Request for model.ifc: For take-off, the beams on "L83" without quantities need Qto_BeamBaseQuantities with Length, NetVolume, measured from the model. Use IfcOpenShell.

First a look at what the model holds.

```python
import ifcopenshell
import ifcopenshell.util.element
import ifcopenshell.util.unit

model = ifcopenshell.open("model.ifc")
print(model.schema)
for unit_type in ("LENGTHUNIT", "AREAUNIT", "VOLUMEUNIT"):
    print(unit_type, ifcopenshell.util.unit.calculate_unit_scale(model, unit_type))
storey = next(s for s in model.by_type("IfcBuildingStorey") if s.Name == "L83")
beams = [e for e in ifcopenshell.util.element.get_decomposition(storey) if e.is_a("IfcBeam")]
for e in sorted(beams, key=lambda e: e.id()):
    print(e.id(), e.is_a(), e.Name, list(ifcopenshell.util.element.get_psets(e, qtos_only=True)), sep=" | ")
```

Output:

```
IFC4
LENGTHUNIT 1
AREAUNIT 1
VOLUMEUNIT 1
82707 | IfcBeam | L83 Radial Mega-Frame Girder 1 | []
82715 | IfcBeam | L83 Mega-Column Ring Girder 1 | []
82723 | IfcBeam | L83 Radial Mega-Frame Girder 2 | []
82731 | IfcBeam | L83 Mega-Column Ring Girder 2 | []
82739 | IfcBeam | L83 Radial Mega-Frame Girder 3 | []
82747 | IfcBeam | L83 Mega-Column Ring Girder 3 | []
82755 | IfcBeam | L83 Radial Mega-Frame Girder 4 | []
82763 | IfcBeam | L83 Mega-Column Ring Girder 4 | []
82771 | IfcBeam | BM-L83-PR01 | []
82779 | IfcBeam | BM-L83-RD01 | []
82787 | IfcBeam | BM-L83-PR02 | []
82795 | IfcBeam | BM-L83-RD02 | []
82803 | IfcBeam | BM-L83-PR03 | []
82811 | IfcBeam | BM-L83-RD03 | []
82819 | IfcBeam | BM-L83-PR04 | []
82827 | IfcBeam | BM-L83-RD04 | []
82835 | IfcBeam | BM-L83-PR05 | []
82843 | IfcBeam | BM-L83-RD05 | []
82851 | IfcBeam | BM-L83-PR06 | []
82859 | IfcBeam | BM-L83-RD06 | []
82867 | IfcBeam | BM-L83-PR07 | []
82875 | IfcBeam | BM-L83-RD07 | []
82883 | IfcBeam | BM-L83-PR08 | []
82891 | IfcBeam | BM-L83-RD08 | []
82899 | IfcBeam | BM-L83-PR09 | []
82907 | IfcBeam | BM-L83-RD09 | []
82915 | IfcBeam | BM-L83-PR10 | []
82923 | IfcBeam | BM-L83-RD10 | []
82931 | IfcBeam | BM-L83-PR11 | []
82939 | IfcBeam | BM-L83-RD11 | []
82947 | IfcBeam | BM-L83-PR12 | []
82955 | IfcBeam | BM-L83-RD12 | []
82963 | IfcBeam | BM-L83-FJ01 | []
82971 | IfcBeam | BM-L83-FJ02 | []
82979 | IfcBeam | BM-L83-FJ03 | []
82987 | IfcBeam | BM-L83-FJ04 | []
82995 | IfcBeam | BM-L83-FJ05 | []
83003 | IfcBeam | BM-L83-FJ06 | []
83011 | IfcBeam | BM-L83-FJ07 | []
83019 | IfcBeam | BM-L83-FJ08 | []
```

```python
import ifcopenshell
import ifcopenshell.api.pset
import ifcopenshell.geom
import ifcopenshell.util.element
import ifcopenshell.util.shape
import ifcopenshell.util.unit

model = ifcopenshell.open("model.ifc")
unit_scale = ifcopenshell.util.unit.calculate_unit_scale(model)
volume_scale = ifcopenshell.util.unit.calculate_unit_scale(model, "VOLUMEUNIT")
settings = ifcopenshell.geom.settings()

storey = next(s for s in model.by_type("IfcBuildingStorey") if s.Name == "L83")
beams = [e for e in ifcopenshell.util.element.get_decomposition(storey) if e.is_a("IfcBeam")]

for e in sorted(beams, key=lambda e: e.id()):
    if ifcopenshell.util.element.get_psets(e, qtos_only=True, should_inherit=False):
        continue
    # Geometry comes back in metres, in the element's own axes.
    shape = ifcopenshell.geom.create_shape(settings, e)
    values = {
        "Length": ifcopenshell.util.shape.get_max_xyz(shape.geometry) / unit_scale,
        "NetVolume": ifcopenshell.util.shape.get_volume(shape.geometry) / volume_scale,
    }
    qto = ifcopenshell.api.pset.add_qto(model, product=e, name="Qto_BeamBaseQuantities")
    ifcopenshell.api.pset.edit_qto(model, qto=qto, properties=values)
    print(e.id(), {k: round(v, 3) for k, v in values.items()})

model.write("model_v2.ifc")
```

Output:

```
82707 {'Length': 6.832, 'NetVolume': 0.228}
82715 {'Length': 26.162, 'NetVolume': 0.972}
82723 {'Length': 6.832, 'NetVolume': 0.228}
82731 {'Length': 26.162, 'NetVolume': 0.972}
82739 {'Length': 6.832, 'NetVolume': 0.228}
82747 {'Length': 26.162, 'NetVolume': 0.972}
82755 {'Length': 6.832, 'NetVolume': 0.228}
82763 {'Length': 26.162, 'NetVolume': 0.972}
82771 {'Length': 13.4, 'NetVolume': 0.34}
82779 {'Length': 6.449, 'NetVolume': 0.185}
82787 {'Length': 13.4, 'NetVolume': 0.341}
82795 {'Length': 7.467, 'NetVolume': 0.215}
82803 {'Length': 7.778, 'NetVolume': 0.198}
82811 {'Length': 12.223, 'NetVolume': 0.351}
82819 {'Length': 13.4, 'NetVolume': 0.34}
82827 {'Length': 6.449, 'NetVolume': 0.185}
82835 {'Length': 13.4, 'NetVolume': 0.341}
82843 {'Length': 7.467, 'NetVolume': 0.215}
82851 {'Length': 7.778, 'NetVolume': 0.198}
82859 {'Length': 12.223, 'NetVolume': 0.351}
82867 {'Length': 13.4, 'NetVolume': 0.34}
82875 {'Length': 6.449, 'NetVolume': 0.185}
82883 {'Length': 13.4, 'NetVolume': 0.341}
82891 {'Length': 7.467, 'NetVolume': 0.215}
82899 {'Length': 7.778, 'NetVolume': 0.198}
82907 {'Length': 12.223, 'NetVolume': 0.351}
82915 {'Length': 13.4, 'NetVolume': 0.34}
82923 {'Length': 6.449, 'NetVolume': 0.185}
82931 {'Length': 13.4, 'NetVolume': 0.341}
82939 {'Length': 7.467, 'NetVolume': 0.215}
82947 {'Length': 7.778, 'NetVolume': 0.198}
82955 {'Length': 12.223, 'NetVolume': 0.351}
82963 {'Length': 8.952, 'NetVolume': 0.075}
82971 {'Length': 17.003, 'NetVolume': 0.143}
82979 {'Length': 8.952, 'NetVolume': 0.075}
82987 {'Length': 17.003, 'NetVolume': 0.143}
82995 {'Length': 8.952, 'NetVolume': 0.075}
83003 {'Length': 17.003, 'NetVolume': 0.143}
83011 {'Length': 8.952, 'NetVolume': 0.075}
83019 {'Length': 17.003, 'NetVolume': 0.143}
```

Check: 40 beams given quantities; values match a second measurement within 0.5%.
